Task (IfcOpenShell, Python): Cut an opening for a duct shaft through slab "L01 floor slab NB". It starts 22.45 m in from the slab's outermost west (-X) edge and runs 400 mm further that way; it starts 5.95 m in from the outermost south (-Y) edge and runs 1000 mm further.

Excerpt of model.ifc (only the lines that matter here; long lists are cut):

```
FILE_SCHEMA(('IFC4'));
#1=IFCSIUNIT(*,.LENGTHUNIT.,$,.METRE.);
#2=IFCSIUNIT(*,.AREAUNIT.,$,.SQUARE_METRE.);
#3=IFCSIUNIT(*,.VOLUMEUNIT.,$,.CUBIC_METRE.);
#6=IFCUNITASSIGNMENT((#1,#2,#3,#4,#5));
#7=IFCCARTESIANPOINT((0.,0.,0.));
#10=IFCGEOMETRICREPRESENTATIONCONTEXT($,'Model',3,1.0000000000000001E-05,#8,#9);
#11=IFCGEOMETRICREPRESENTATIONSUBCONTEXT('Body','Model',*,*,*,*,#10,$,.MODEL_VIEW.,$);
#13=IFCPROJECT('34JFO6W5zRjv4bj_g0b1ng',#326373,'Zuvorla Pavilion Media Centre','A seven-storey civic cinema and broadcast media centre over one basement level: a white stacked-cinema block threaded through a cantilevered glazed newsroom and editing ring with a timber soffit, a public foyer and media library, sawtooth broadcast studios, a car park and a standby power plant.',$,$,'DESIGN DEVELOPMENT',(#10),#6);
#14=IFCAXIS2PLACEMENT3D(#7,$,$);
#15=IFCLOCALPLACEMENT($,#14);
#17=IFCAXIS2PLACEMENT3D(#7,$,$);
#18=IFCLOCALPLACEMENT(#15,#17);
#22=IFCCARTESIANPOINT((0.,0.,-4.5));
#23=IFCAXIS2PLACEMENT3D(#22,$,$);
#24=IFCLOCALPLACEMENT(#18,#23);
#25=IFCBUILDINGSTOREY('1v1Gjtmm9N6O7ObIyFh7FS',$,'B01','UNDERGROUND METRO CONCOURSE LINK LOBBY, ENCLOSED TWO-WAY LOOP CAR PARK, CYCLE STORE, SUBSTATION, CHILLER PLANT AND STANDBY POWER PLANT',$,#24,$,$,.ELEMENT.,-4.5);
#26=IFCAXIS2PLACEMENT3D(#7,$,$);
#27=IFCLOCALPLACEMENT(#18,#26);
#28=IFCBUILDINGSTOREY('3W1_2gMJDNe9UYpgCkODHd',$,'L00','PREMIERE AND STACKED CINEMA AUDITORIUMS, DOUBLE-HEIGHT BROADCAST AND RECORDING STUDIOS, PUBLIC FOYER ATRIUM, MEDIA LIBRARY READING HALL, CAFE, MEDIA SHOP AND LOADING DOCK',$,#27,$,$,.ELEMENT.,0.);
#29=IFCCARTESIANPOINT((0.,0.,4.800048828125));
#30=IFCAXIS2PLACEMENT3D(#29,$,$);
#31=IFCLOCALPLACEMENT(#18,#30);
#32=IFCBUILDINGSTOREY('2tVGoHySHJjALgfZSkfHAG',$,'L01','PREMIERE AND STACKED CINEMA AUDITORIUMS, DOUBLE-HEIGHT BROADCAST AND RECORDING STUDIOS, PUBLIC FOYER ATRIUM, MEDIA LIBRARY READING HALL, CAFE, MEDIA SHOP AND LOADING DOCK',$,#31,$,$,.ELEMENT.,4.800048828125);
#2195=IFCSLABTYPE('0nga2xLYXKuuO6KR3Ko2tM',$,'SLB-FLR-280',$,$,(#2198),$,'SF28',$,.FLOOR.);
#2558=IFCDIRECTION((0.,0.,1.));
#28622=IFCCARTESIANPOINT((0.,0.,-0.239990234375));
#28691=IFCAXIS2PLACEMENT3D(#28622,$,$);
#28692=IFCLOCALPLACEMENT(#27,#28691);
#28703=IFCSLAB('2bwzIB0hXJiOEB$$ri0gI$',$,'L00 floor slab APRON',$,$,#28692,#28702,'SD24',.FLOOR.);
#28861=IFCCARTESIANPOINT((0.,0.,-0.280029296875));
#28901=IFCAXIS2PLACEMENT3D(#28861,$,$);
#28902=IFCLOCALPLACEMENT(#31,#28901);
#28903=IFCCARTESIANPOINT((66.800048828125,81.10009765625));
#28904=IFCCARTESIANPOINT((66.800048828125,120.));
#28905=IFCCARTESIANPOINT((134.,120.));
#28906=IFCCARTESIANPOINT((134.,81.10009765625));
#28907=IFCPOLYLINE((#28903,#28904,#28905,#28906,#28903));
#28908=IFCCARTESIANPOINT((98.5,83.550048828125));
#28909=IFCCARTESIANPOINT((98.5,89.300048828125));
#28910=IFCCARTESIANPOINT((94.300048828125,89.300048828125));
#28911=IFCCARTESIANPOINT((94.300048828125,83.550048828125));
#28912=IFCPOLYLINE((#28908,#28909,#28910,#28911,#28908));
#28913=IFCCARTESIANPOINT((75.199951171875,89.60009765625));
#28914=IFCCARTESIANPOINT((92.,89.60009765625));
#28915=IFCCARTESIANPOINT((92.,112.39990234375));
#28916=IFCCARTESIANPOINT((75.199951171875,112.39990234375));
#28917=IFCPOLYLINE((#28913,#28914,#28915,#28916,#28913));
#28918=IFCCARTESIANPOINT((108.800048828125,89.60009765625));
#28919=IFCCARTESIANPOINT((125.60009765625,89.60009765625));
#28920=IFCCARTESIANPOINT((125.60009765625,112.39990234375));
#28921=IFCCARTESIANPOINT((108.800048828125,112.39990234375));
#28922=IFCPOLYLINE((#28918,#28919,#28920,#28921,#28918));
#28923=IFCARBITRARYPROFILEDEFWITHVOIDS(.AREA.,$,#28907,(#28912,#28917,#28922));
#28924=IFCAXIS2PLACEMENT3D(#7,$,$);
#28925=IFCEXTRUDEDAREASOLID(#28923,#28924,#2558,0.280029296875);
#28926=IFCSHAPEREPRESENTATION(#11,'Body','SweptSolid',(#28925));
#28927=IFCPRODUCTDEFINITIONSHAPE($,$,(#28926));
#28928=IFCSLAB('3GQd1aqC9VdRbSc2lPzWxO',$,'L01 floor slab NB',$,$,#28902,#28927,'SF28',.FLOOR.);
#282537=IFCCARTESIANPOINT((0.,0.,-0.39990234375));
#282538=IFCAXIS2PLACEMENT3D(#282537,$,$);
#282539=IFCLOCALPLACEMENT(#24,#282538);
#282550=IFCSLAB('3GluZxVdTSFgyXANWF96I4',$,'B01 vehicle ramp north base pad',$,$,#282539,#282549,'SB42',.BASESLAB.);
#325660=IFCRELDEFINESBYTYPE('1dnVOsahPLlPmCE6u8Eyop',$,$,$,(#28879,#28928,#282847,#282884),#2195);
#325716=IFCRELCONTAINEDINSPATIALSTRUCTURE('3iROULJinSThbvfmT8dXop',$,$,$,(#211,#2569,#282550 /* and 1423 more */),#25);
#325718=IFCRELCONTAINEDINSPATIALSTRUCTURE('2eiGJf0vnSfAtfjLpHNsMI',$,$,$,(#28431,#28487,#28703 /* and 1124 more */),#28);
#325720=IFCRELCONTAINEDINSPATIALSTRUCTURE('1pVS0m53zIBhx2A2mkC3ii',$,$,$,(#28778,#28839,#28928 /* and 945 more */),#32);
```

```python
import numpy as np
import ifcopenshell
import ifcopenshell.api.feature
import ifcopenshell.api.geometry
import ifcopenshell.api.root
import ifcopenshell.geom
import ifcopenshell.util.placement
import ifcopenshell.util.representation
import ifcopenshell.util.shape
import ifcopenshell.util.unit

model = ifcopenshell.open("model.ifc")
unit_scale = ifcopenshell.util.unit.calculate_unit_scale(model)
settings = ifcopenshell.geom.settings()


def volume(element):
    """Net volume in cubic metres, openings subtracted."""
    shape = ifcopenshell.geom.create_shape(settings, element)
    return ifcopenshell.util.shape.get_volume(shape.geometry)


slab = model.by_id(28928)
before = volume(slab)

# Extent in the slab's own axes, in metres. The edges named are its -X and -Y sides.
slab_shape = ifcopenshell.geom.create_shape(settings, slab)
vertices = ifcopenshell.util.shape.get_vertices(slab_shape.geometry)
x_min, y_min, bottom = vertices.min(axis=0)
top = vertices[:, 2].max()

opening = ifcopenshell.api.root.create_entity(model, ifc_class="IfcOpeningElement", name="Duct shaft opening", predefined_type="OPENING")
context = ifcopenshell.util.representation.get_context(model, "Model", "Body", "MODEL_VIEW")
width, depth = 0.4, 1
outline = [(0.0, 0.0), (width, 0.0), (width, depth), (0.0, depth), (0.0, 0.0)]
# Overshoot both faces by 50 mm so the cut is clean.
shape = ifcopenshell.api.geometry.add_slab_representation(
    model, context=context, depth=top - bottom + 0.1, polyline=outline
)
ifcopenshell.api.geometry.assign_representation(model, product=opening, representation=shape)

matrix = ifcopenshell.util.placement.get_local_placement(slab.ObjectPlacement)
matrix[:, 3] = matrix @ np.append(np.array([x_min + 22.45, y_min + 5.95, bottom - 0.05]) / unit_scale, 1.0)
ifcopenshell.api.geometry.edit_object_placement(model, product=opening, matrix=matrix, is_si=False)
ifcopenshell.api.feature.add_feature(model, feature=opening, element=slab)

after = volume(slab)

print(f"slab volume {before:.3f} -> {after:.3f} m3")

model.write("model_edited.ifc")
```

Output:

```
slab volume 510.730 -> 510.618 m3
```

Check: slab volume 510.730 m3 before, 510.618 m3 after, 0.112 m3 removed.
